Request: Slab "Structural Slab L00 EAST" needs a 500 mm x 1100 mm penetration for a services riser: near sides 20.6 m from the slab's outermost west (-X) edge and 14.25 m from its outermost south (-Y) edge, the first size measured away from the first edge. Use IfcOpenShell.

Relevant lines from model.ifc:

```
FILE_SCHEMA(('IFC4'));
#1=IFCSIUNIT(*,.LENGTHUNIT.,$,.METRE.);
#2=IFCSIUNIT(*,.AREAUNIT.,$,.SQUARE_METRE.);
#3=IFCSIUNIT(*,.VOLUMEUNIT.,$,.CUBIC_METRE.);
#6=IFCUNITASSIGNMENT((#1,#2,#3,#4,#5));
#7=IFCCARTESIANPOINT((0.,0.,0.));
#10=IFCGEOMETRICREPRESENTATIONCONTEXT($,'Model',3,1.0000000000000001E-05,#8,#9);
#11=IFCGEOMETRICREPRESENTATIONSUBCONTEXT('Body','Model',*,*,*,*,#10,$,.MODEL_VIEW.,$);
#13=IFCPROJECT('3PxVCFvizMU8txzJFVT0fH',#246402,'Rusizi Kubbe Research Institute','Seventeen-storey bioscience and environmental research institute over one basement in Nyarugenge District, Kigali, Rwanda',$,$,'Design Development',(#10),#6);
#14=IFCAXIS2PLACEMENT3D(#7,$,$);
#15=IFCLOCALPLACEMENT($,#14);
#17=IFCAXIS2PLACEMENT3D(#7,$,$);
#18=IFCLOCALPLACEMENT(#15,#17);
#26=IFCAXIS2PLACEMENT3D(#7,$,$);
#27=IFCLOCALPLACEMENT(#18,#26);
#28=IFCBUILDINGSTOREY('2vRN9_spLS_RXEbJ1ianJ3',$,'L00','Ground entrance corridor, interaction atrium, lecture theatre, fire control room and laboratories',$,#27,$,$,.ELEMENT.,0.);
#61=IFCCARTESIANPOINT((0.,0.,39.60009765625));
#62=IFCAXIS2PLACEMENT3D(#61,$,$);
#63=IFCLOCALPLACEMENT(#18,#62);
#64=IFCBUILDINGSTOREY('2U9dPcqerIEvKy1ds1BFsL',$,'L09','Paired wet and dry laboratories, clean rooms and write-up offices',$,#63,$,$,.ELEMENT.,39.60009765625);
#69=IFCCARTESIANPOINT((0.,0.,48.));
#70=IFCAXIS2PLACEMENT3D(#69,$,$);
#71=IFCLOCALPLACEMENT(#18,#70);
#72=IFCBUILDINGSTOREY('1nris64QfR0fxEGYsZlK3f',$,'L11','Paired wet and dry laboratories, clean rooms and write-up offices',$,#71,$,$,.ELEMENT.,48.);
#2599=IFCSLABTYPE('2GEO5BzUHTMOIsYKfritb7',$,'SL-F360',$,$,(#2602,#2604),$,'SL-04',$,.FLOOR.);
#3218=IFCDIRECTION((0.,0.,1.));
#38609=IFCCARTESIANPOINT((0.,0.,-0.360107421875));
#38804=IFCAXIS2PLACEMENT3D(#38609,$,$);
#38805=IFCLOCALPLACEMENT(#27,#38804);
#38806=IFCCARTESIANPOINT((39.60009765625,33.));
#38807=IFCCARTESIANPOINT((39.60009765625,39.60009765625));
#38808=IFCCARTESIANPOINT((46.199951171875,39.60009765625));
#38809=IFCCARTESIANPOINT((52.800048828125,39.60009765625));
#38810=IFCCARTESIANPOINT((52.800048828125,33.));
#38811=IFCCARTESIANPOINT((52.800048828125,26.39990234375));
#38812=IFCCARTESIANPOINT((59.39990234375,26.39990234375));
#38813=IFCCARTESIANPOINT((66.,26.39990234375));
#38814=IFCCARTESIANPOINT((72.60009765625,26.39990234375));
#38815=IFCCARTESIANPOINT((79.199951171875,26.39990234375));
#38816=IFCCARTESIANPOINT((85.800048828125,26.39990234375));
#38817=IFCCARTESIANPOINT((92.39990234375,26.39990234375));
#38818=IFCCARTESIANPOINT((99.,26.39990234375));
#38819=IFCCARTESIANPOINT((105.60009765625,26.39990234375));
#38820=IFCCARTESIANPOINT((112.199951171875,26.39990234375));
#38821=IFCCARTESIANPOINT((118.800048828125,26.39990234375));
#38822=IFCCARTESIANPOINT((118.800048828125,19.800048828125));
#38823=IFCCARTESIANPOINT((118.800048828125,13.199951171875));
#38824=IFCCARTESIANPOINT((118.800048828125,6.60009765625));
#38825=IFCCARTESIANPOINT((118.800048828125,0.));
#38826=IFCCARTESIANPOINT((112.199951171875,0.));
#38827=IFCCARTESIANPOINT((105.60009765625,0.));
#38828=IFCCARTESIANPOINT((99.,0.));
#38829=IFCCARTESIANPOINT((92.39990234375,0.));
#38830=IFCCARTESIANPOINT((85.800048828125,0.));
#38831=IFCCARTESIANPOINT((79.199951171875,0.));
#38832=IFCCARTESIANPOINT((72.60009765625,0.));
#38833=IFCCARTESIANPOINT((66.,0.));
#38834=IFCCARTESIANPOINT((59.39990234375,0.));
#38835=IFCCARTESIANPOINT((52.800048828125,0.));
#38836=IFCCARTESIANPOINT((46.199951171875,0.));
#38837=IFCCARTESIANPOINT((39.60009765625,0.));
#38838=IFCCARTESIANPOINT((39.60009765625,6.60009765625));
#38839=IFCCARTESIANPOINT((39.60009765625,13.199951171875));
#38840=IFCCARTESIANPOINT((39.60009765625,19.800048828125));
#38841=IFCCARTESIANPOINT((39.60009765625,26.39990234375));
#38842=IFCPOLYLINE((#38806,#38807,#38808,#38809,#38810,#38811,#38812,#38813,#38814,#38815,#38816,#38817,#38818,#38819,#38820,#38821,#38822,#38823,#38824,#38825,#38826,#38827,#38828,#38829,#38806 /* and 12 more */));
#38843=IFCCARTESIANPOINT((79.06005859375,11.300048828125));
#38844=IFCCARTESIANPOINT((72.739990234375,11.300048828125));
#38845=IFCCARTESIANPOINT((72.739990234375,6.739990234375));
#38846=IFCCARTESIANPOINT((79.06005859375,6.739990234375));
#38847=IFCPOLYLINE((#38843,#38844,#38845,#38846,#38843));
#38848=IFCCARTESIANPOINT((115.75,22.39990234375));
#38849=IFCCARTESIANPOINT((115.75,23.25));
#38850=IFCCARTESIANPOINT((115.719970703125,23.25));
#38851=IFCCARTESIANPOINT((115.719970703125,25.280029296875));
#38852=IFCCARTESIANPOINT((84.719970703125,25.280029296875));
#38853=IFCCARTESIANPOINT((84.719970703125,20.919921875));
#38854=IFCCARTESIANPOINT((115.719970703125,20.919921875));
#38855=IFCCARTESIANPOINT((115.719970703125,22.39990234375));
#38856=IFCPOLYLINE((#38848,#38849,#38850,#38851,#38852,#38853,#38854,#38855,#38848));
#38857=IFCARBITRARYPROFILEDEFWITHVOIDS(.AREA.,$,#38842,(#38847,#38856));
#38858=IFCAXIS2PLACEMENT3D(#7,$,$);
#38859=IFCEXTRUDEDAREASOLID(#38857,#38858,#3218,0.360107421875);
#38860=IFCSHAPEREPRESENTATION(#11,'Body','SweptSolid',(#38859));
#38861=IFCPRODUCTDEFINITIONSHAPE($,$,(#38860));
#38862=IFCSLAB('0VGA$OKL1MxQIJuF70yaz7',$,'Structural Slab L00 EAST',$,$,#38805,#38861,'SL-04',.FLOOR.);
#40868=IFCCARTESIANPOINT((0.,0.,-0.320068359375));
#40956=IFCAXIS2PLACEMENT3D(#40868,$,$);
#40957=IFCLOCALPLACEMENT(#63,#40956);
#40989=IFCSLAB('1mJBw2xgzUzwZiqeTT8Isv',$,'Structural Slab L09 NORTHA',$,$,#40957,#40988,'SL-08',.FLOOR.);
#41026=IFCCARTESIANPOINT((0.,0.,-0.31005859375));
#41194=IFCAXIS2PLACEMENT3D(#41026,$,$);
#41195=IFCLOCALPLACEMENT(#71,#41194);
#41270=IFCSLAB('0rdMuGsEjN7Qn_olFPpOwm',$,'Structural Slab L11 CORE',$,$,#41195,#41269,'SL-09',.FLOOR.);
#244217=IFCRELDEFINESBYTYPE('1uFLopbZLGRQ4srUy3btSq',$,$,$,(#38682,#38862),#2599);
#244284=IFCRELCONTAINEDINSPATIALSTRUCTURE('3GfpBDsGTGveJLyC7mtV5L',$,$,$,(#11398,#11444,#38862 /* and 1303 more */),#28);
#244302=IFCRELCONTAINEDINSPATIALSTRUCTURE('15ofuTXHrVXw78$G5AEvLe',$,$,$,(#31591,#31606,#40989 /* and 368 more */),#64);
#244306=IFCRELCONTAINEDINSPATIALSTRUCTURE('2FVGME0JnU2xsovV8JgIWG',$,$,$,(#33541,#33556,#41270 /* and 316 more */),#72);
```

```python
import numpy as np
import ifcopenshell
import ifcopenshell.api.feature
import ifcopenshell.api.geometry
import ifcopenshell.api.root
import ifcopenshell.geom
import ifcopenshell.util.placement
import ifcopenshell.util.representation
import ifcopenshell.util.shape
import ifcopenshell.util.unit

model = ifcopenshell.open("model.ifc")
unit_scale = ifcopenshell.util.unit.calculate_unit_scale(model)
settings = ifcopenshell.geom.settings()


def volume(element):
    """Net volume in cubic metres, openings subtracted."""
    shape = ifcopenshell.geom.create_shape(settings, element)
    return ifcopenshell.util.shape.get_volume(shape.geometry)


slab = model.by_guid("0VGA$OKL1MxQIJuF70yaz7")
before = volume(slab)

# Extent in the slab's own axes, in metres. The edges named are its -X and -Y sides.
slab_shape = ifcopenshell.geom.create_shape(settings, slab)
vertices = ifcopenshell.util.shape.get_vertices(slab_shape.geometry)
x_min, y_min, bottom = vertices.min(axis=0)
top = vertices[:, 2].max()

opening = ifcopenshell.api.root.create_entity(model, ifc_class="IfcOpeningElement", name="Services riser opening", predefined_type="OPENING")
context = ifcopenshell.util.representation.get_context(model, "Model", "Body", "MODEL_VIEW")
width, depth = 0.5, 1.1
outline = [(0.0, 0.0), (width, 0.0), (width, depth), (0.0, depth), (0.0, 0.0)]
# Overshoot both faces by 50 mm so the cut is clean.
shape = ifcopenshell.api.geometry.add_slab_representation(
    model, context=context, depth=top - bottom + 0.1, polyline=outline
)
ifcopenshell.api.geometry.assign_representation(model, product=opening, representation=shape)

matrix = ifcopenshell.util.placement.get_local_placement(slab.ObjectPlacement)
matrix[:, 3] = matrix @ np.append(np.array([x_min + 20.6, y_min + 14.25, bottom - 0.05]) / unit_scale, 1.0)
ifcopenshell.api.geometry.edit_object_placement(model, product=opening, matrix=matrix, is_si=False)
ifcopenshell.api.feature.add_feature(model, feature=opening, element=slab)

after = volume(slab)

print(f"slab volume {before:.3f} -> {after:.3f} m3")

model.write("model-out.ifc")
```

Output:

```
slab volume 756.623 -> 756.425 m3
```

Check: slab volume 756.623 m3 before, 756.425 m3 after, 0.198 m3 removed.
